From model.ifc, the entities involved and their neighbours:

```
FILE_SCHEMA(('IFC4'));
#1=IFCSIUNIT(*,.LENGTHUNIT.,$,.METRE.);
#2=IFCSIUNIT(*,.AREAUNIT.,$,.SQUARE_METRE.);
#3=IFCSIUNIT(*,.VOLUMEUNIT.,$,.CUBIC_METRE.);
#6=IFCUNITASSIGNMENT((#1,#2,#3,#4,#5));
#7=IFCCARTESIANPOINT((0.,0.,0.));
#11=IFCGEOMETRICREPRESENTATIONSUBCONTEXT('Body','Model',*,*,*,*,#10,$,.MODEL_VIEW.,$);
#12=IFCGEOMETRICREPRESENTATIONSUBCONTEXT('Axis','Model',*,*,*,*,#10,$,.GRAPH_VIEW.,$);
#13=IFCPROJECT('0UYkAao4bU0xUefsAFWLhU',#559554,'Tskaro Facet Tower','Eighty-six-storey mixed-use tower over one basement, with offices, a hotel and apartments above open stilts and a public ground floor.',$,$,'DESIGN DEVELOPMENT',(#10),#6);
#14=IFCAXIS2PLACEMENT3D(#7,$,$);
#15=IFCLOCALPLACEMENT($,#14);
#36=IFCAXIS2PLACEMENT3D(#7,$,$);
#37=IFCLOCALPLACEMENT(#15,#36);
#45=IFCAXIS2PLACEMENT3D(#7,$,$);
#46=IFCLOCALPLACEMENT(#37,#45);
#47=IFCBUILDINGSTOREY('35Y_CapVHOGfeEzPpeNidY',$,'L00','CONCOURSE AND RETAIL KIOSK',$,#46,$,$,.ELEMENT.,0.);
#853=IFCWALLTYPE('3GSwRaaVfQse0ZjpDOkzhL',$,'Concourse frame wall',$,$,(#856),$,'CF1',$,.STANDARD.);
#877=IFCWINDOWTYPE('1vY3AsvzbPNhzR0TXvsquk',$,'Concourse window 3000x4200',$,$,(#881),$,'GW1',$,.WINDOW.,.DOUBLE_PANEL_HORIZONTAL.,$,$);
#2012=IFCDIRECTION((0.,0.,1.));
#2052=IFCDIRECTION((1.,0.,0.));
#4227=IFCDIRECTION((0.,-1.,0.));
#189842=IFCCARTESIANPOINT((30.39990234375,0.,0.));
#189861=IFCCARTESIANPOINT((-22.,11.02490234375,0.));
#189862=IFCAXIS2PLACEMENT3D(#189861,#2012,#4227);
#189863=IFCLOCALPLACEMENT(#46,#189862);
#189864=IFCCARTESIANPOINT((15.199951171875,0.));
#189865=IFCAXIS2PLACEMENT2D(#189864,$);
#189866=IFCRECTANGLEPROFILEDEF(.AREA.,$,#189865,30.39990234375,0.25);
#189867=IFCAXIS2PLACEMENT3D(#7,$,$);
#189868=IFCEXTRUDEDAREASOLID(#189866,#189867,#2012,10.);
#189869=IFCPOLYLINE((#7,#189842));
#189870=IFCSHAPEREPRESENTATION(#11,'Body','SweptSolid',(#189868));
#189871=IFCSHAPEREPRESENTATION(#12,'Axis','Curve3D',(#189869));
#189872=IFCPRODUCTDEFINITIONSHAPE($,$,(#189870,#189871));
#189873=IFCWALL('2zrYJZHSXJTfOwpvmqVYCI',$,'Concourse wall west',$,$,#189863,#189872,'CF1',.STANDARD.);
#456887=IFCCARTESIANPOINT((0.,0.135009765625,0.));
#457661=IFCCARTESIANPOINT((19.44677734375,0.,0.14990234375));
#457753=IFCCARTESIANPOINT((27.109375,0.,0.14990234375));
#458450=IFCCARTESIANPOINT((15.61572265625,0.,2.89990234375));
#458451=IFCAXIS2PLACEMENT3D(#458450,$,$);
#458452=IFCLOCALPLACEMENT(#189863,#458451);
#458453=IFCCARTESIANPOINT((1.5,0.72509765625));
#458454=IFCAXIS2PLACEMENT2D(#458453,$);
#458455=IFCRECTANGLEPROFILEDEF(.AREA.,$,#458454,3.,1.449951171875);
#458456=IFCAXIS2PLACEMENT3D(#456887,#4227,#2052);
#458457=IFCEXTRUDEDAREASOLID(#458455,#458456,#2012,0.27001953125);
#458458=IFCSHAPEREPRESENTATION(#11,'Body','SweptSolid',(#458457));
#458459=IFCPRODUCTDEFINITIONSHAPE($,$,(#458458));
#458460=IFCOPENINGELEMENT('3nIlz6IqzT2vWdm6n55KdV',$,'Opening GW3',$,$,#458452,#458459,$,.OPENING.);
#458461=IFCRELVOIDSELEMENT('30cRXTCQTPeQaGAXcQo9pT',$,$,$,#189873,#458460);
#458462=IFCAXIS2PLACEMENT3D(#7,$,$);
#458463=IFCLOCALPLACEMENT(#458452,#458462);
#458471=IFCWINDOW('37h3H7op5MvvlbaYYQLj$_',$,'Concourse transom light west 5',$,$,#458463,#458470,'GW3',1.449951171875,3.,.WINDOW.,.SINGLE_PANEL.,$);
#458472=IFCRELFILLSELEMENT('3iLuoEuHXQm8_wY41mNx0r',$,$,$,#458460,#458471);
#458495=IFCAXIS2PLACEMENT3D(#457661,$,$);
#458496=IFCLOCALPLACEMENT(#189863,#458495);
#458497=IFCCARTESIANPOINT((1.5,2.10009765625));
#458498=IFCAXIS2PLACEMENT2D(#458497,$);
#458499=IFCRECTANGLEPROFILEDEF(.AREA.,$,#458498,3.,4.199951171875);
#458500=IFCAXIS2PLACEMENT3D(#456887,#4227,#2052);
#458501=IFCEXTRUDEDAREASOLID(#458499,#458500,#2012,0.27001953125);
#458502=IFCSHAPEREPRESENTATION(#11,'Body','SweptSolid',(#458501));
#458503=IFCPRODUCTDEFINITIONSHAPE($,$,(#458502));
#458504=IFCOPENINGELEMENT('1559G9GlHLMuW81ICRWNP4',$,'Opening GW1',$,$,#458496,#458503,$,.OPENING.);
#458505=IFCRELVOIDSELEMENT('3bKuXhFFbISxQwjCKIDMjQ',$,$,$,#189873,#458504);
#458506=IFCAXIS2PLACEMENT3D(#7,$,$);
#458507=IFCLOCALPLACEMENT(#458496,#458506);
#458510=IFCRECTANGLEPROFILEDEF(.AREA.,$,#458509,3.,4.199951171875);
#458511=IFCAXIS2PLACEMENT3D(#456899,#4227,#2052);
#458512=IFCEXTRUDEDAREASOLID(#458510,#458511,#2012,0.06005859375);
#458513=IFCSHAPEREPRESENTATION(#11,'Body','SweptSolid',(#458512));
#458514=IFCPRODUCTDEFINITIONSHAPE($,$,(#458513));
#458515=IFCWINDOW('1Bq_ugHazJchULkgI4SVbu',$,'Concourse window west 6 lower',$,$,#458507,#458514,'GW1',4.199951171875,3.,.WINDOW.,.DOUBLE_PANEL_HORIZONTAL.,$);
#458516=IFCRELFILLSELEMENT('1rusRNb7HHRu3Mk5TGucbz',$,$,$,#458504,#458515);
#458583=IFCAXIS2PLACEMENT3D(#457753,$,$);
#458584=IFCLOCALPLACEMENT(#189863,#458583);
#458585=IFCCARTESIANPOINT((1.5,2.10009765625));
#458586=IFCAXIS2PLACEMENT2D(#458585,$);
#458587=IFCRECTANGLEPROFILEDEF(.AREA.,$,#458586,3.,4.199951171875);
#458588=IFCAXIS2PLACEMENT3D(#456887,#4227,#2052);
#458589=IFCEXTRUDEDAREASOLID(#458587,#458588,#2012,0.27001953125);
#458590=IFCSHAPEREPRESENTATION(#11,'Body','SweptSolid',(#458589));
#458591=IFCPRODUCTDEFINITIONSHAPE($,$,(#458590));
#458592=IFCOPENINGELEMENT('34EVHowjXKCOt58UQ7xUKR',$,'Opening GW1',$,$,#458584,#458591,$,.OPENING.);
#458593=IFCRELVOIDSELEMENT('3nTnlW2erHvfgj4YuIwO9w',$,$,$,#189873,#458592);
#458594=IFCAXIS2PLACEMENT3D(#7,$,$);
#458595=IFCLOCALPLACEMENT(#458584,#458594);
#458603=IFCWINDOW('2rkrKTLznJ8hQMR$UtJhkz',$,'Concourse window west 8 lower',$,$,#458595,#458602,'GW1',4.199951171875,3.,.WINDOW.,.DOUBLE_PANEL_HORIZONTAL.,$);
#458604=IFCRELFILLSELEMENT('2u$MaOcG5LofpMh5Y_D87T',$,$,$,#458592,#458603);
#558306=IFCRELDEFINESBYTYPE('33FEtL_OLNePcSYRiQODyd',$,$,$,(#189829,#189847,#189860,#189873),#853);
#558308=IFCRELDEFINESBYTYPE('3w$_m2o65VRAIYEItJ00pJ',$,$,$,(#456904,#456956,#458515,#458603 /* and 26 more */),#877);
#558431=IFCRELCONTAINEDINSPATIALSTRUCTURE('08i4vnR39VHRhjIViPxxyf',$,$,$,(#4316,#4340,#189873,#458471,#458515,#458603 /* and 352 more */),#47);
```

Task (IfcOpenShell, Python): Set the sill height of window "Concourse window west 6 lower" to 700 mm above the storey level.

```python
import numpy as np
import ifcopenshell
import ifcopenshell.api.geometry
import ifcopenshell.geom
import ifcopenshell.util.element
import ifcopenshell.util.placement
import ifcopenshell.util.shape
import ifcopenshell.util.unit

model = ifcopenshell.open("model.ifc")
unit_scale = ifcopenshell.util.unit.calculate_unit_scale(model)

window = model.by_guid("1Bq_ugHazJchULkgI4SVbu")
opening = window.FillsVoids[0].RelatingOpeningElement
storey = ifcopenshell.util.element.get_container(window, ifc_class="IfcBuildingStorey")
level = ifcopenshell.util.placement.get_local_placement(storey.ObjectPlacement)[2, 3]

# The opening's origin need not be at the sill, so measure its lowest point.
shape = ifcopenshell.geom.create_shape(ifcopenshell.geom.settings(), opening)
bottom = ifcopenshell.util.shape.get_shape_bottom_elevation(shape, shape.geometry) / unit_scale
dz = level + 0.7 / unit_scale - bottom

shift = np.array([0.0, 0.0, dz])
# The window is placed relative to its opening, so it follows when the opening moves.
matrix = ifcopenshell.util.placement.get_local_placement(opening.ObjectPlacement)
matrix[:3, 3] += shift
ifcopenshell.api.geometry.edit_object_placement(
    model, product=opening, matrix=matrix, is_si=False, should_transform_children=True
)

print(f"moved by {dz * unit_scale:+.3f} m")

model.write("model_edited.ifc")
```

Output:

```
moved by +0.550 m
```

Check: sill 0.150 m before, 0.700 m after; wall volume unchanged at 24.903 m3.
